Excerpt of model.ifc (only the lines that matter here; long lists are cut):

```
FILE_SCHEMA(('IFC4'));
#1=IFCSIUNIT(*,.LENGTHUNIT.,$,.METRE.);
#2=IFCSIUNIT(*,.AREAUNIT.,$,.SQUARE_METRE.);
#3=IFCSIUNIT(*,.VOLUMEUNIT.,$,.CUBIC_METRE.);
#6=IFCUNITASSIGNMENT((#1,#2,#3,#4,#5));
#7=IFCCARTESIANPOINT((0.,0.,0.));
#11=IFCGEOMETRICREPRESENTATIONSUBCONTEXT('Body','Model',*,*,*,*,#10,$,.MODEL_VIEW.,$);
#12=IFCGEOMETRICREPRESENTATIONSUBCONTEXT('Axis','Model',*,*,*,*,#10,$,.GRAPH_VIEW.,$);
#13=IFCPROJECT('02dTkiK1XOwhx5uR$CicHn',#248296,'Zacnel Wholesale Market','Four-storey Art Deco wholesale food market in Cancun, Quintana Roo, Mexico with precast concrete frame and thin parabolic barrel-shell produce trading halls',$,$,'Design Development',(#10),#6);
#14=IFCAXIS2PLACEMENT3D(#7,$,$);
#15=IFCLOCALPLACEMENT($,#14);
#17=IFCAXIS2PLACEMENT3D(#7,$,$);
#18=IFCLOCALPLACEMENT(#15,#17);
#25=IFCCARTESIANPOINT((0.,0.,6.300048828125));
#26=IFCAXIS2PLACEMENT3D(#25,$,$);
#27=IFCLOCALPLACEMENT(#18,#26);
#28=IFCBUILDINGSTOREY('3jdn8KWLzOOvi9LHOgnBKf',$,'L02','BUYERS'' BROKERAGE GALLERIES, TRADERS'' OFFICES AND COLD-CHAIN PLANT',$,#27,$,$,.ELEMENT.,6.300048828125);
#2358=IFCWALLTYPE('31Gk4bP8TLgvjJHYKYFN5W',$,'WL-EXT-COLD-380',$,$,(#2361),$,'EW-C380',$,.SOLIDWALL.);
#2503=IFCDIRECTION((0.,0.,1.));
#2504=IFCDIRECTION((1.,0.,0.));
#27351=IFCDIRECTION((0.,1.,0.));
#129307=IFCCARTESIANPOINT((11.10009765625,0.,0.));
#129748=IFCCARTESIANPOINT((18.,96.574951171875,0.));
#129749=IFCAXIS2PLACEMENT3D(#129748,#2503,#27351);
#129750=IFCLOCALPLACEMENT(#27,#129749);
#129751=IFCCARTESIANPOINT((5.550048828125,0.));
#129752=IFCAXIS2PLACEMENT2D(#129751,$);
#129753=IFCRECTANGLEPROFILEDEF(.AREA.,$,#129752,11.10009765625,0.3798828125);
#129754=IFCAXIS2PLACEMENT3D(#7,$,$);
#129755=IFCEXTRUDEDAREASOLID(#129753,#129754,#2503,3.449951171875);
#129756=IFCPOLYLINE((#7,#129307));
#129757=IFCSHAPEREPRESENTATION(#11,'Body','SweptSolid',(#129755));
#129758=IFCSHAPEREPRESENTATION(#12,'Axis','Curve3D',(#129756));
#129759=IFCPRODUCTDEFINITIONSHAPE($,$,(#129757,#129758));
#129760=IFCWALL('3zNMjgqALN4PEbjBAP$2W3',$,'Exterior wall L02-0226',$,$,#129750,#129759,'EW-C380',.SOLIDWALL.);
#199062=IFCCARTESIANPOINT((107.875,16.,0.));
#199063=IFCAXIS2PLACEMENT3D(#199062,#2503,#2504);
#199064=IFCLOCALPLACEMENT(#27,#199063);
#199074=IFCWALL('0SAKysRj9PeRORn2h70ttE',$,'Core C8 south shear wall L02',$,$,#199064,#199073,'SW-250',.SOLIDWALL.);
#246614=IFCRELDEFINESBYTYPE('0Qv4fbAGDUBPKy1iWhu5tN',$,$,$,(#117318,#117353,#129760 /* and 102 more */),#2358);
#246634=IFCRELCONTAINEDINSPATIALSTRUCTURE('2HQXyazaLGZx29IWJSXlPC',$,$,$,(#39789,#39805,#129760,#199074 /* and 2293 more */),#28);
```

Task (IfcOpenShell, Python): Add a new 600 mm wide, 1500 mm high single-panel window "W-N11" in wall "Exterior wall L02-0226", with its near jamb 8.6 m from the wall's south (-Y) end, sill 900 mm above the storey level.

```python
import numpy as np
import ifcopenshell
import ifcopenshell.api.feature
import ifcopenshell.api.geometry
import ifcopenshell.api.root
import ifcopenshell.api.spatial
import ifcopenshell.geom
import ifcopenshell.util.element
import ifcopenshell.util.placement
import ifcopenshell.util.representation
import ifcopenshell.util.shape
import ifcopenshell.util.unit

model = ifcopenshell.open("model.ifc")
unit_scale = ifcopenshell.util.unit.calculate_unit_scale(model)
settings = ifcopenshell.geom.settings()


def volume(element):
    """Net volume in cubic metres, openings subtracted."""
    shape = ifcopenshell.geom.create_shape(settings, element)
    return ifcopenshell.util.shape.get_volume(shape.geometry)


wall = model.by_guid("3zNMjgqALN4PEbjBAP$2W3")
storey = ifcopenshell.util.element.get_container(wall, ifc_class="IfcBuildingStorey")
context = ifcopenshell.util.representation.get_context(model, "Model", "Body", "MODEL_VIEW")
before = volume(wall)

width, height, from_end, sill = 0.6, 1.5, 8.6, 0.9  # metres

# The wall runs along its own X axis, and the end named is its -X end.
wall_shape = ifcopenshell.geom.create_shape(settings, wall)
x, y, z = ifcopenshell.util.shape.get_vertices(wall_shape.geometry).T
start = x.min() + from_end
face, thickness = float(y.min()), float(y.max() - y.min())
wall_matrix = ifcopenshell.util.placement.get_local_placement(wall.ObjectPlacement)
level = ifcopenshell.util.placement.get_local_placement(storey.ObjectPlacement)[2, 3]


def in_wall(x, y):
    """Placement at x, y metres in the wall's axes, at sill height."""
    matrix = wall_matrix.copy()
    matrix[:, 3] = wall_matrix @ np.array([x / unit_scale, y / unit_scale, 0.0, 1.0])
    matrix[2, 3] = level + sill / unit_scale
    return matrix


# Opening: a box that overshoots both wall faces by 50 mm.
opening = ifcopenshell.api.root.create_entity(model, ifc_class="IfcOpeningElement", predefined_type="OPENING")
box = ifcopenshell.api.geometry.add_wall_representation(
    model, context=context, length=width, height=height, thickness=thickness + 0.1
)
ifcopenshell.api.geometry.assign_representation(model, product=opening, representation=box)
ifcopenshell.api.geometry.edit_object_placement(model, product=opening, matrix=in_wall(start, face - 0.05), is_si=False)
ifcopenshell.api.feature.add_feature(model, feature=opening, element=wall)

window = ifcopenshell.api.root.create_entity(model, ifc_class="IfcWindow", name="W-N11", predefined_type="WINDOW")
window.OverallWidth, window.OverallHeight = width / unit_scale, height / unit_scale
window.PartitioningType = "SINGLE_PANEL"
body = ifcopenshell.api.geometry.add_window_representation(
    model,
    context=context,
    overall_width=window.OverallWidth,
    overall_height=window.OverallHeight,
    partition_type="SINGLE_PANEL",
)
ifcopenshell.api.geometry.assign_representation(model, product=window, representation=body)
ifcopenshell.api.spatial.assign_container(model, products=[window], relating_structure=storey)
ifcopenshell.api.feature.add_filling(model, opening=opening, element=window)

# Centre the window in the wall's thickness.
ifcopenshell.api.geometry.edit_object_placement(model, product=window, matrix=in_wall(start, face), is_si=False)
window_shape = ifcopenshell.geom.create_shape(settings, window)
depth = ifcopenshell.util.shape.get_vertices(window_shape.geometry)[:, 1]
offset = face + thickness / 2 - (depth.min() + depth.max()) / 2
ifcopenshell.api.geometry.edit_object_placement(model, product=window, matrix=in_wall(start, offset), is_si=False)

after = volume(wall)

print(f"wall volume {before:.3f} -> {after:.3f} m3")

model.write("model-out.ifc")
```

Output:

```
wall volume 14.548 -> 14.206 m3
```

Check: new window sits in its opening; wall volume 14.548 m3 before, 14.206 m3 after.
